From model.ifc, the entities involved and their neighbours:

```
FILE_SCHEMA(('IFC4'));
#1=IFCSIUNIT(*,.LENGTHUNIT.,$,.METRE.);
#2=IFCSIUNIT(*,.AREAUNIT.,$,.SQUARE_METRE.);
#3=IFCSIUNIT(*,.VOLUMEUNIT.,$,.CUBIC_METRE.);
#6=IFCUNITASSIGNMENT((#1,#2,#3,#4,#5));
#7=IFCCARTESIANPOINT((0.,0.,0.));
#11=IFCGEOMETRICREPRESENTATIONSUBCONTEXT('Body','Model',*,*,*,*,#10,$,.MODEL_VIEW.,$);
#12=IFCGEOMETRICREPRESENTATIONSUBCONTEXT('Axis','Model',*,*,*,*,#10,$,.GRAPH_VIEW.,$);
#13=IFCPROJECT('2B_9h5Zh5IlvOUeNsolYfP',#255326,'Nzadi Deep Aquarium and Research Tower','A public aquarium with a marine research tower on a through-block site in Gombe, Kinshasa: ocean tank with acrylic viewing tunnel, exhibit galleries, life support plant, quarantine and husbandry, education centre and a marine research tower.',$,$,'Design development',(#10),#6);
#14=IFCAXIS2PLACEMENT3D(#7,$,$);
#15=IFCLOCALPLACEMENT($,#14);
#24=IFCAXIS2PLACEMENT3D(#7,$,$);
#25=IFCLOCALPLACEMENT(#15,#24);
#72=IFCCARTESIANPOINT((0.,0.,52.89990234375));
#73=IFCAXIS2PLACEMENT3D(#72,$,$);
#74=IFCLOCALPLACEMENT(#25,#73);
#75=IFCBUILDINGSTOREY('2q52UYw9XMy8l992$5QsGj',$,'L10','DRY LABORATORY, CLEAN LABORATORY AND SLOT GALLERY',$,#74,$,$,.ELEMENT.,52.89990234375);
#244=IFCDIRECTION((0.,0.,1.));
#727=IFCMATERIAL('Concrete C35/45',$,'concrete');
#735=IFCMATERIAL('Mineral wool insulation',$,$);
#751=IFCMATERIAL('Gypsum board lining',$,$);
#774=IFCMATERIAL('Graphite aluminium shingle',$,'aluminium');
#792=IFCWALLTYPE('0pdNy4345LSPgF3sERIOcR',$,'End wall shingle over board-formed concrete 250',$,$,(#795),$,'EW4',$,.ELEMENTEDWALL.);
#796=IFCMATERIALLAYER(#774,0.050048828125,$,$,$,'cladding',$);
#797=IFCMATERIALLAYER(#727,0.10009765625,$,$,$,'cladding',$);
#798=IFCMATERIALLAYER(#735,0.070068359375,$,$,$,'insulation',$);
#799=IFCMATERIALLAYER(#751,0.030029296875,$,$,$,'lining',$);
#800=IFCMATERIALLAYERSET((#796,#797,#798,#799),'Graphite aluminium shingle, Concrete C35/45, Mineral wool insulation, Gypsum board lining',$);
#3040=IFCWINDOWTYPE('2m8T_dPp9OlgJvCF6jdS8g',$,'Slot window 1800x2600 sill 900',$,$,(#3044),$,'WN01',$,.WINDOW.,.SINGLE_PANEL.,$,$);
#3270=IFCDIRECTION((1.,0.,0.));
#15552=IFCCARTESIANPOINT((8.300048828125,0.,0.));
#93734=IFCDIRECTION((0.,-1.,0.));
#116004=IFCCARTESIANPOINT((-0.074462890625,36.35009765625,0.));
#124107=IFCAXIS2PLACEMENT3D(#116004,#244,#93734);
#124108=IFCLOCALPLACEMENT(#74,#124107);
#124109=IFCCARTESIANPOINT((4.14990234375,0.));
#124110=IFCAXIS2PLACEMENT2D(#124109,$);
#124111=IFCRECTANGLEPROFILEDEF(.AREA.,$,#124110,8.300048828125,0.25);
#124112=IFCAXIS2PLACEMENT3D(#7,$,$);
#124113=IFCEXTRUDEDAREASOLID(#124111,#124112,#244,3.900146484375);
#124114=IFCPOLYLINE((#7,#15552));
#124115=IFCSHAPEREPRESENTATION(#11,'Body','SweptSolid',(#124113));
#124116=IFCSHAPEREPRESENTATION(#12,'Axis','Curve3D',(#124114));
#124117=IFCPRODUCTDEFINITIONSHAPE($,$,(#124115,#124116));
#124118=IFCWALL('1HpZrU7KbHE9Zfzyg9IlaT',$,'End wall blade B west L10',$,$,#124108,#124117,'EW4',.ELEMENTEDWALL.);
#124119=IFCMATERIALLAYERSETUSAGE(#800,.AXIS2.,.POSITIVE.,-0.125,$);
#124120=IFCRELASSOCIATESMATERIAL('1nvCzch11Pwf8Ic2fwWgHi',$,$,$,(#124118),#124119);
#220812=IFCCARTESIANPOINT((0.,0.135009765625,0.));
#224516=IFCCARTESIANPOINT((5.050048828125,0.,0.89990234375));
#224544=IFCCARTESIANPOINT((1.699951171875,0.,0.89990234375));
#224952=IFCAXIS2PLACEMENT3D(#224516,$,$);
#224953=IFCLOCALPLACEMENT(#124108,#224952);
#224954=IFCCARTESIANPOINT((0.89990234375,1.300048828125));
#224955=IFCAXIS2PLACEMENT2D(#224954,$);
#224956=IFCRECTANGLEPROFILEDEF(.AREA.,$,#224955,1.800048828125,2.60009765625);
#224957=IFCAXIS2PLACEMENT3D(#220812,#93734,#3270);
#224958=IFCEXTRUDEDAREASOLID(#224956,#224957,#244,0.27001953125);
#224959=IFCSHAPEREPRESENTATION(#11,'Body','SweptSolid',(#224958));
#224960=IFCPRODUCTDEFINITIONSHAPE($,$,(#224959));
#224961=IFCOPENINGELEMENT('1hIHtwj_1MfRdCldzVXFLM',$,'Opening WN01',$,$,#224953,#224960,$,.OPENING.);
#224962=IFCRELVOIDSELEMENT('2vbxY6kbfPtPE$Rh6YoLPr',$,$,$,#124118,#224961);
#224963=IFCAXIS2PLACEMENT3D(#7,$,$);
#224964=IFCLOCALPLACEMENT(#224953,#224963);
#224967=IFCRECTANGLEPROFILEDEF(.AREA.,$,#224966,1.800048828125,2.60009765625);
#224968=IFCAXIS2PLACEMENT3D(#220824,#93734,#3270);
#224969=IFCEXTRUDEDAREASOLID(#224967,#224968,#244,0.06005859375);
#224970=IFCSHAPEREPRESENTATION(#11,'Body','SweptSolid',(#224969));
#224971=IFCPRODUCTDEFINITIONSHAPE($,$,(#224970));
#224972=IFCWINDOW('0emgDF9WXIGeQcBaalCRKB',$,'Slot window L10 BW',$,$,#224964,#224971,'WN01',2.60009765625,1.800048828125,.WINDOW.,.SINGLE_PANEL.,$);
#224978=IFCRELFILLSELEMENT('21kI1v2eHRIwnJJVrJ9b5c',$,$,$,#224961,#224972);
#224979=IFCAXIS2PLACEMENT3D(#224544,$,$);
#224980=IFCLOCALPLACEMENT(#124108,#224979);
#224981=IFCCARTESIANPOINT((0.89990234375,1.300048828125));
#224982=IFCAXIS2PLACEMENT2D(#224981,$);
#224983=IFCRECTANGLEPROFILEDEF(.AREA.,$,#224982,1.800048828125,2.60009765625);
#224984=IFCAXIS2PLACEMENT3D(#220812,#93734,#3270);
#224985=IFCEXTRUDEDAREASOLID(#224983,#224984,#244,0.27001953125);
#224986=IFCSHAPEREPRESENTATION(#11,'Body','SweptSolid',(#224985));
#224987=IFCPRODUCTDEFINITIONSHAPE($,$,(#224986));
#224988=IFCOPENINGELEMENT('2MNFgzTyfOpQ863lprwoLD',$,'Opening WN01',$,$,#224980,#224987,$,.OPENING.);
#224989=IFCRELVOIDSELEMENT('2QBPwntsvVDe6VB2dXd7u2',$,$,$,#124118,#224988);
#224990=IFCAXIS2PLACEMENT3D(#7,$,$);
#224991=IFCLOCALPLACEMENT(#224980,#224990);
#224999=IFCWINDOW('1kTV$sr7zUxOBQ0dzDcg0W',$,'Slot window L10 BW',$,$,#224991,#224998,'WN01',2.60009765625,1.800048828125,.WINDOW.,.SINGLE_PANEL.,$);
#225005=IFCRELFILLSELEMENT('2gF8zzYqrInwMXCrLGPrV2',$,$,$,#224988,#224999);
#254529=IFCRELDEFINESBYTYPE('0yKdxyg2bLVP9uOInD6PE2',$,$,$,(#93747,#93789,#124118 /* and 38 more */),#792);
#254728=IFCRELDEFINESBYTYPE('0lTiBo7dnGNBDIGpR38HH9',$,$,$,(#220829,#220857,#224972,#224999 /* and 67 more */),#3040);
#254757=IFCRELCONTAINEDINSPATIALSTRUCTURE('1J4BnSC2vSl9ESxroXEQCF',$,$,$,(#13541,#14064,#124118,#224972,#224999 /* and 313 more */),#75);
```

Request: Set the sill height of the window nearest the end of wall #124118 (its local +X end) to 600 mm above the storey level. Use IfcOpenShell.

```python
import numpy as np
import ifcopenshell
import ifcopenshell.api.geometry
import ifcopenshell.geom
import ifcopenshell.util.element
import ifcopenshell.util.placement
import ifcopenshell.util.shape
import ifcopenshell.util.unit

model = ifcopenshell.open("model.ifc")
unit_scale = ifcopenshell.util.unit.calculate_unit_scale(model)

window = model.by_guid("0emgDF9WXIGeQcBaalCRKB")
opening = window.FillsVoids[0].RelatingOpeningElement
storey = ifcopenshell.util.element.get_container(window, ifc_class="IfcBuildingStorey")
level = ifcopenshell.util.placement.get_local_placement(storey.ObjectPlacement)[2, 3]

# The opening's origin need not be at the sill, so measure its lowest point.
shape = ifcopenshell.geom.create_shape(ifcopenshell.geom.settings(), opening)
bottom = ifcopenshell.util.shape.get_shape_bottom_elevation(shape, shape.geometry) / unit_scale
dz = level + 0.6 / unit_scale - bottom

shift = np.array([0.0, 0.0, dz])
# The window is placed relative to its opening, so it follows when the opening moves.
matrix = ifcopenshell.util.placement.get_local_placement(opening.ObjectPlacement)
matrix[:3, 3] += shift
ifcopenshell.api.geometry.edit_object_placement(
    model, product=opening, matrix=matrix, is_si=False, should_transform_children=True
)

print(f"moved by {dz * unit_scale:+.3f} m")

model.write("model_v2.ifc")
```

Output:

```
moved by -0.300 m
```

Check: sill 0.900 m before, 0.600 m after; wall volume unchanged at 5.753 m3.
